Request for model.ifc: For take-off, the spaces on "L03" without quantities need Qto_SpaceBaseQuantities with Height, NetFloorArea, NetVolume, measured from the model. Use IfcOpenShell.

First a look at what the model holds.

```python
import ifcopenshell
import ifcopenshell.util.element
import ifcopenshell.util.unit

model = ifcopenshell.open("model.ifc")
print(model.schema)
for unit_type in ("LENGTHUNIT", "AREAUNIT", "VOLUMEUNIT"):
    print(unit_type, ifcopenshell.util.unit.calculate_unit_scale(model, unit_type))
storey = next(s for s in model.by_type("IfcBuildingStorey") if s.Name == "L03")
spaces = [e for e in ifcopenshell.util.element.get_decomposition(storey) if e.is_a("IfcSpace")]
for e in sorted(spaces, key=lambda e: e.id()):
    print(e.id(), e.is_a(), e.Name, list(ifcopenshell.util.element.get_psets(e, qtos_only=True)), sep=" | ")
```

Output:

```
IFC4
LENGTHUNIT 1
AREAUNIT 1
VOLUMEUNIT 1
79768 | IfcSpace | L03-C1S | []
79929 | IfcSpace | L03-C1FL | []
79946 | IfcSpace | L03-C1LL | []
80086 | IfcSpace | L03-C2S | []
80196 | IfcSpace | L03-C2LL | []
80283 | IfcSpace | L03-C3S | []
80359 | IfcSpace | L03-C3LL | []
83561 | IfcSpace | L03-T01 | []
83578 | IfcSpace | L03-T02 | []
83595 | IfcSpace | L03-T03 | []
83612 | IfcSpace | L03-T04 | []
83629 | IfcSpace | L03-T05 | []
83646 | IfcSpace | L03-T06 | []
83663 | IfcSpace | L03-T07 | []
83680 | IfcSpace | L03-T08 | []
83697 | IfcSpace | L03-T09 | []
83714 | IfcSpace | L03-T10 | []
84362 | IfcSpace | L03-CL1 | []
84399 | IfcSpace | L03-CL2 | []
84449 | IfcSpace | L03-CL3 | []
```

```python
import ifcopenshell
import ifcopenshell.api.pset
import ifcopenshell.geom
import ifcopenshell.util.element
import ifcopenshell.util.shape
import ifcopenshell.util.unit

model = ifcopenshell.open("model.ifc")
unit_scale = ifcopenshell.util.unit.calculate_unit_scale(model)
area_scale = ifcopenshell.util.unit.calculate_unit_scale(model, "AREAUNIT")
volume_scale = ifcopenshell.util.unit.calculate_unit_scale(model, "VOLUMEUNIT")
settings = ifcopenshell.geom.settings()

storey = next(s for s in model.by_type("IfcBuildingStorey") if s.Name == "L03")
spaces = [e for e in ifcopenshell.util.element.get_decomposition(storey) if e.is_a("IfcSpace")]

for e in sorted(spaces, key=lambda e: e.id()):
    if ifcopenshell.util.element.get_psets(e, qtos_only=True, should_inherit=False):
        continue
    # Geometry comes back in metres, in the element's own axes.
    shape = ifcopenshell.geom.create_shape(settings, e)
    values = {
        "Height": ifcopenshell.util.shape.get_z(shape.geometry) / unit_scale,
        "NetFloorArea": ifcopenshell.util.shape.get_footprint_area(shape.geometry) / area_scale,
        "NetVolume": ifcopenshell.util.shape.get_volume(shape.geometry) / volume_scale,
    }
    qto = ifcopenshell.api.pset.add_qto(model, product=e, name="Qto_SpaceBaseQuantities")
    ifcopenshell.api.pset.edit_qto(model, qto=qto, properties=values)
    print(e.id(), {k: round(v, 3) for k, v in values.items()})

model.write("model_v2.ifc")
```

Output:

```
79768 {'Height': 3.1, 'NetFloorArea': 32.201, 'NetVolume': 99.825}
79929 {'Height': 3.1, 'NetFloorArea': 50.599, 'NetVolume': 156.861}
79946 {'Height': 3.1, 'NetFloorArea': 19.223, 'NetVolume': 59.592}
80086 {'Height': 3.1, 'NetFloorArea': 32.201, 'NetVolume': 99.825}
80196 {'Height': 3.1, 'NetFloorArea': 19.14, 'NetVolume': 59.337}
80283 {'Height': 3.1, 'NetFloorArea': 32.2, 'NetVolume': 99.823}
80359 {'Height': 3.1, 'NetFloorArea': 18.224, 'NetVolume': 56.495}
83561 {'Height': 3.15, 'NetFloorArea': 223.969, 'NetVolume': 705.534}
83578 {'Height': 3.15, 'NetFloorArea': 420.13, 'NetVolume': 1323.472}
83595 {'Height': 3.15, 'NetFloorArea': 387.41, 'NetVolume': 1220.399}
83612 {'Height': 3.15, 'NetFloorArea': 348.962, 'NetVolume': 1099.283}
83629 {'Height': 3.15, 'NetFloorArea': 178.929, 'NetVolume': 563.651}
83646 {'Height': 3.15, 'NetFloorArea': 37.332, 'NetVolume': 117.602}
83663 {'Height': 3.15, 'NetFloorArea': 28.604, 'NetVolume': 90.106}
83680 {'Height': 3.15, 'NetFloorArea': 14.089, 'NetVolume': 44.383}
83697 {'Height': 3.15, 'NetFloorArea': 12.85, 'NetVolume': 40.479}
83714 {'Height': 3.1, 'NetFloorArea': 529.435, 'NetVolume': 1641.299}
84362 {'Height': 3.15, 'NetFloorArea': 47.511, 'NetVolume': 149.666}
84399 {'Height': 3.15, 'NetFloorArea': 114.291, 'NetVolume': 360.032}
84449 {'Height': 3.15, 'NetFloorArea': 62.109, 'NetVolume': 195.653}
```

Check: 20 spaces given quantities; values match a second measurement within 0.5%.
